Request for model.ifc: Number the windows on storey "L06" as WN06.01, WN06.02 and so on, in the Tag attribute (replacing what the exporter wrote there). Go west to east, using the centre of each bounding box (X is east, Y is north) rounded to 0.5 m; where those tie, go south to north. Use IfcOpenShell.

First a look at what the model holds.

```python
import ifcopenshell
import ifcopenshell.util.element
import ifcopenshell.util.placement

model = ifcopenshell.open("model.ifc")
print(model.schema)
storey = next(s for s in model.by_type("IfcBuildingStorey") if s.Name == "L06")
windows = [e for e in ifcopenshell.util.element.get_decomposition(storey) if e.is_a("IfcWindow")]
for e in sorted(windows, key=lambda e: e.id()):
    origin = ifcopenshell.util.placement.get_local_placement(e.ObjectPlacement)[:3, 3]
    print(e.id(), e.Tag, e.Name, origin.round(2) + 0.0, sep=" | ")
```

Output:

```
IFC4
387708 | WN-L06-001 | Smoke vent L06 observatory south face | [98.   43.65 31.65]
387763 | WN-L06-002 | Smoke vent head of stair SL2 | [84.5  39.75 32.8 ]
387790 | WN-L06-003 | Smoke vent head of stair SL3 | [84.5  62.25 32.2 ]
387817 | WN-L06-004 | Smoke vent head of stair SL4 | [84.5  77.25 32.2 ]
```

```python
import ifcopenshell
import ifcopenshell.geom
import ifcopenshell.util.element
import ifcopenshell.util.shape

model = ifcopenshell.open("model.ifc")
settings = ifcopenshell.geom.settings()
settings.set("use-world-coords", True)


def centre(element):
    shape = ifcopenshell.geom.create_shape(settings, element)
    return ifcopenshell.util.shape.get_bbox_centroid(shape.geometry)


storey = next(s for s in model.by_type("IfcBuildingStorey") if s.Name == "L06")
windows = [e for e in ifcopenshell.util.element.get_decomposition(storey) if e.is_a("IfcWindow")]

# Insertion points can sit at a corner or the storey origin, so sort by the geometry (in metres).
centres = {e: centre(e) for e in windows}
windows.sort(key=lambda e: (round(centres[e][0] / 0.5), centres[e][1]))

for i, e in enumerate(windows, start=1):
    number = f"WN06.{i:02d}"
    e.Tag = number
    print(e.id(), number)

model.write("model-out.ifc")
```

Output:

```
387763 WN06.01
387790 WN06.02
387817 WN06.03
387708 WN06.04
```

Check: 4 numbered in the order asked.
